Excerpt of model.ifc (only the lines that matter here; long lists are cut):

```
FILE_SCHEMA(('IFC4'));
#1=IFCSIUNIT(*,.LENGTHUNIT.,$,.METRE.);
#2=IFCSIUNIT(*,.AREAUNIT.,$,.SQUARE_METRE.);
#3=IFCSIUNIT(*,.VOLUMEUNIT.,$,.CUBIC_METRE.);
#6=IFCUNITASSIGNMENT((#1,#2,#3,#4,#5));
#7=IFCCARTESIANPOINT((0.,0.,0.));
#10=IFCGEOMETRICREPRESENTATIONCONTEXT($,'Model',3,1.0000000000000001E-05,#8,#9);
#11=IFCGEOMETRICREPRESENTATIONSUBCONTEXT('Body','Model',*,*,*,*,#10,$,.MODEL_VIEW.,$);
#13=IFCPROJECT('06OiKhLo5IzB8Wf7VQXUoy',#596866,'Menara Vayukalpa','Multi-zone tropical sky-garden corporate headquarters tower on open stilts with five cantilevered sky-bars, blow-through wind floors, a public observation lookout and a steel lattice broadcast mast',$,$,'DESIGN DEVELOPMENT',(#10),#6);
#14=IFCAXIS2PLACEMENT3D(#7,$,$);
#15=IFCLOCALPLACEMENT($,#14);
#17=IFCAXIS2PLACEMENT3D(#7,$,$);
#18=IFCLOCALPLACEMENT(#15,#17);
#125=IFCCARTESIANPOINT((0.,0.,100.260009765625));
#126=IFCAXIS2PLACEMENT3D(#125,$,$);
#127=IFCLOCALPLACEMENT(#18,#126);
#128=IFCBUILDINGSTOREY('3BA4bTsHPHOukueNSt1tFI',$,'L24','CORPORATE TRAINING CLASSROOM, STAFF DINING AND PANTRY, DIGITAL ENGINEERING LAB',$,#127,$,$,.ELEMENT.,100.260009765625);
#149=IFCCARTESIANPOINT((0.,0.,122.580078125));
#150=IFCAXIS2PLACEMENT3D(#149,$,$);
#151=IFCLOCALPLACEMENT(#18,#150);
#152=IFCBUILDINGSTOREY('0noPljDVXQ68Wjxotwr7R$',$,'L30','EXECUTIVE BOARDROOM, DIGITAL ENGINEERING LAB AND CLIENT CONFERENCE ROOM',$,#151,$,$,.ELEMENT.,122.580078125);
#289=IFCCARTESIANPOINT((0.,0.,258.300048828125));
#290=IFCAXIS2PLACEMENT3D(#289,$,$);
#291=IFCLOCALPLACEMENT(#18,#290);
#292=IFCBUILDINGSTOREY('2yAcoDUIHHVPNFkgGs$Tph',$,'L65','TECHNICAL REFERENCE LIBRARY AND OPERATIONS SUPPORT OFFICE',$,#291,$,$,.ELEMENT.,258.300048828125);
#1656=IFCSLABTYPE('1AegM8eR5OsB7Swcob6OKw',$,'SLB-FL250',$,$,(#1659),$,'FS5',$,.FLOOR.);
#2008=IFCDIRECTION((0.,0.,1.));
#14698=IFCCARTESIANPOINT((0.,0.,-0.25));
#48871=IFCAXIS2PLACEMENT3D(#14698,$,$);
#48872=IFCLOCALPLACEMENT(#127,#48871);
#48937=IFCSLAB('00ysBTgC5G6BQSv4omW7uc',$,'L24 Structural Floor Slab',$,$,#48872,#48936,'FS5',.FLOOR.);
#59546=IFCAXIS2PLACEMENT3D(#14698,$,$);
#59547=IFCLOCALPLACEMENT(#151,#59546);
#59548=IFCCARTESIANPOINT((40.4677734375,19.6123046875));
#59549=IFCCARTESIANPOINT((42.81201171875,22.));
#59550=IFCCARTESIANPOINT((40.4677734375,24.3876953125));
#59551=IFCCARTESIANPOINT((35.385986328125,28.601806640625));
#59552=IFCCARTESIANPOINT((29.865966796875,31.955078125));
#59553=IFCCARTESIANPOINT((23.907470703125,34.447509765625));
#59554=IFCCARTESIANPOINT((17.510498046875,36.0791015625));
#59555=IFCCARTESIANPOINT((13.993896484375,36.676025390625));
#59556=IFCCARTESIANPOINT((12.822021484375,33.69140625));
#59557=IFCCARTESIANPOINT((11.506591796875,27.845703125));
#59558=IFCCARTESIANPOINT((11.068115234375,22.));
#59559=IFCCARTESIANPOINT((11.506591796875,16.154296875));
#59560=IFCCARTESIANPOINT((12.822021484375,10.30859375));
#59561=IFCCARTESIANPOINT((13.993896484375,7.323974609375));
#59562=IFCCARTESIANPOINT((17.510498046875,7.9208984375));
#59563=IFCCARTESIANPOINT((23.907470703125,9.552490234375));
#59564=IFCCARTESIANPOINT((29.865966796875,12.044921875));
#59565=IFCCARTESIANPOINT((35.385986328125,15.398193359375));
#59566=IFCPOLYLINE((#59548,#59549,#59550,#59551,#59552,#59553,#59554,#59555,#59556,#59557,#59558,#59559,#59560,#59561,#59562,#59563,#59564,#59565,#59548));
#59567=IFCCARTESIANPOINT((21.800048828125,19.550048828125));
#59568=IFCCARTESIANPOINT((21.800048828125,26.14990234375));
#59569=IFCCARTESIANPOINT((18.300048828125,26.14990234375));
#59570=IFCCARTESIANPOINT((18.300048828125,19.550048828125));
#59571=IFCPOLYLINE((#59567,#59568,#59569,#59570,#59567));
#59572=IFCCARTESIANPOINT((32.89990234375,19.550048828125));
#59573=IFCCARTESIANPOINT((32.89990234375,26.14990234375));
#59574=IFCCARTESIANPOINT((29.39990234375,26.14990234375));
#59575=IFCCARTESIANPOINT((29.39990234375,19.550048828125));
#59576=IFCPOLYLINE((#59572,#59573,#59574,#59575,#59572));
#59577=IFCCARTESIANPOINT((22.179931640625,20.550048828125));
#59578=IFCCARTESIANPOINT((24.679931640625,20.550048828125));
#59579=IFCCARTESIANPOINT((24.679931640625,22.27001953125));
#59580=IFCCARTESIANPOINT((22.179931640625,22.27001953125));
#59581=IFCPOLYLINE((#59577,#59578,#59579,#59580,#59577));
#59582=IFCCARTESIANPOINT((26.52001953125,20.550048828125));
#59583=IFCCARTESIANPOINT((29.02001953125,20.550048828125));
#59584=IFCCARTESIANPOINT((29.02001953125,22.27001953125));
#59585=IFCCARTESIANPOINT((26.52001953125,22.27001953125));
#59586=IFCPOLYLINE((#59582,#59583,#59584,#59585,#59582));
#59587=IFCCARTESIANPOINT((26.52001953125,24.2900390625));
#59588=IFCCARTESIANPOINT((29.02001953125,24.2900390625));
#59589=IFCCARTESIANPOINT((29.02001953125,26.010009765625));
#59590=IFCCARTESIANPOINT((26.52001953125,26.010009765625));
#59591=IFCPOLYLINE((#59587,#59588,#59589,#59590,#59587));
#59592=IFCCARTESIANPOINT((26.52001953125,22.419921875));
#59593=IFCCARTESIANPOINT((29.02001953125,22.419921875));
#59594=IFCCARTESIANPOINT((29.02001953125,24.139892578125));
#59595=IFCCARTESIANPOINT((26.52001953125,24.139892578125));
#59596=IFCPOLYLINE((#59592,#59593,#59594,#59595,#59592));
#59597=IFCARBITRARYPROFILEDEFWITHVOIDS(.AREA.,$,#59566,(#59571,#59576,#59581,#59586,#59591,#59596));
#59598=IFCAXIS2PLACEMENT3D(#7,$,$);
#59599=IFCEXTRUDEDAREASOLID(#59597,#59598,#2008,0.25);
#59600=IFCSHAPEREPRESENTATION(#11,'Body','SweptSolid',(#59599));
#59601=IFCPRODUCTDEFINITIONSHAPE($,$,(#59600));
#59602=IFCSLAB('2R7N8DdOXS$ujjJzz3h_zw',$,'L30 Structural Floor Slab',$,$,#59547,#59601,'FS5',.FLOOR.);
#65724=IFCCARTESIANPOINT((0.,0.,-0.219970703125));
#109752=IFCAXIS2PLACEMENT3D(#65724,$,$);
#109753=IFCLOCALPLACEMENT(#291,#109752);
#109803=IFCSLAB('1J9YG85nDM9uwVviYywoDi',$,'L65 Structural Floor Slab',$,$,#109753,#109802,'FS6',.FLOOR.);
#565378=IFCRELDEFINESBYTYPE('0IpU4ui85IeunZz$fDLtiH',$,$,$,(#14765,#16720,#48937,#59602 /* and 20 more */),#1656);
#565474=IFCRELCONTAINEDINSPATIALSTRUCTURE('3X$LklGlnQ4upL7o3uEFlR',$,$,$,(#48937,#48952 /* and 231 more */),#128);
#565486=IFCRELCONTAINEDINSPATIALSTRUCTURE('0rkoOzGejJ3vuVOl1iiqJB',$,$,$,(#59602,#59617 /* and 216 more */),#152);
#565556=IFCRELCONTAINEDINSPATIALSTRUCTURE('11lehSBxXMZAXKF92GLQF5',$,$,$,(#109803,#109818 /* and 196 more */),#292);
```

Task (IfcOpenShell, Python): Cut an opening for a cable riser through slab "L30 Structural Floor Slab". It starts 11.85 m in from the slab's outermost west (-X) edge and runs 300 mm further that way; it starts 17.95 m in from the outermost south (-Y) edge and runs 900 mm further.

```python
import numpy as np
import ifcopenshell
import ifcopenshell.api.feature
import ifcopenshell.api.geometry
import ifcopenshell.api.root
import ifcopenshell.geom
import ifcopenshell.util.placement
import ifcopenshell.util.representation
import ifcopenshell.util.shape
import ifcopenshell.util.unit

model = ifcopenshell.open("model.ifc")
unit_scale = ifcopenshell.util.unit.calculate_unit_scale(model)
settings = ifcopenshell.geom.settings()


def volume(element):
    """Net volume in cubic metres, openings subtracted."""
    shape = ifcopenshell.geom.create_shape(settings, element)
    return ifcopenshell.util.shape.get_volume(shape.geometry)


slab = model.by_guid("2R7N8DdOXS$ujjJzz3h_zw")
before = volume(slab)

# Extent in the slab's own axes, in metres. The edges named are its -X and -Y sides.
slab_shape = ifcopenshell.geom.create_shape(settings, slab)
vertices = ifcopenshell.util.shape.get_vertices(slab_shape.geometry)
x_min, y_min, bottom = vertices.min(axis=0)
top = vertices[:, 2].max()

opening = ifcopenshell.api.root.create_entity(model, ifc_class="IfcOpeningElement", name="Cable riser opening", predefined_type="OPENING")
context = ifcopenshell.util.representation.get_context(model, "Model", "Body", "MODEL_VIEW")
width, depth = 0.3, 0.9
outline = [(0.0, 0.0), (width, 0.0), (width, depth), (0.0, depth), (0.0, 0.0)]
# Overshoot both faces by 50 mm so the cut is clean.
shape = ifcopenshell.api.geometry.add_slab_representation(
    model, context=context, depth=top - bottom + 0.1, polyline=outline
)
ifcopenshell.api.geometry.assign_representation(model, product=opening, representation=shape)

matrix = ifcopenshell.util.placement.get_local_placement(slab.ObjectPlacement)
matrix[:, 3] = matrix @ np.append(np.array([x_min + 11.85, y_min + 17.95, bottom - 0.05]) / unit_scale, 1.0)
ifcopenshell.api.geometry.edit_object_placement(model, product=opening, matrix=matrix, is_si=False)
ifcopenshell.api.feature.add_feature(model, feature=opening, element=slab)

after = volume(slab)

print(f"slab volume {before:.3f} -> {after:.3f} m3")

model.write("model_rev.ifc")
```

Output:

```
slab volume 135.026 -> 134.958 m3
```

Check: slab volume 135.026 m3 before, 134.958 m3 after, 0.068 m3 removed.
